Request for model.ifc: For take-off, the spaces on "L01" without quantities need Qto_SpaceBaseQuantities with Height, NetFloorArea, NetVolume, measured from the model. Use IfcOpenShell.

First a look at what the model holds.

```python
import ifcopenshell
import ifcopenshell.util.element
import ifcopenshell.util.unit

model = ifcopenshell.open("model.ifc")
print(model.schema)
for unit_type in ("LENGTHUNIT", "AREAUNIT", "VOLUMEUNIT"):
    print(unit_type, ifcopenshell.util.unit.calculate_unit_scale(model, unit_type))
storey = next(s for s in model.by_type("IfcBuildingStorey") if s.Name == "L01")
spaces = [e for e in ifcopenshell.util.element.get_decomposition(storey) if e.is_a("IfcSpace")]
for e in sorted(spaces, key=lambda e: e.id()):
    print(e.id(), e.is_a(), e.Name, list(ifcopenshell.util.element.get_psets(e, qtos_only=True)), sep=" | ")
```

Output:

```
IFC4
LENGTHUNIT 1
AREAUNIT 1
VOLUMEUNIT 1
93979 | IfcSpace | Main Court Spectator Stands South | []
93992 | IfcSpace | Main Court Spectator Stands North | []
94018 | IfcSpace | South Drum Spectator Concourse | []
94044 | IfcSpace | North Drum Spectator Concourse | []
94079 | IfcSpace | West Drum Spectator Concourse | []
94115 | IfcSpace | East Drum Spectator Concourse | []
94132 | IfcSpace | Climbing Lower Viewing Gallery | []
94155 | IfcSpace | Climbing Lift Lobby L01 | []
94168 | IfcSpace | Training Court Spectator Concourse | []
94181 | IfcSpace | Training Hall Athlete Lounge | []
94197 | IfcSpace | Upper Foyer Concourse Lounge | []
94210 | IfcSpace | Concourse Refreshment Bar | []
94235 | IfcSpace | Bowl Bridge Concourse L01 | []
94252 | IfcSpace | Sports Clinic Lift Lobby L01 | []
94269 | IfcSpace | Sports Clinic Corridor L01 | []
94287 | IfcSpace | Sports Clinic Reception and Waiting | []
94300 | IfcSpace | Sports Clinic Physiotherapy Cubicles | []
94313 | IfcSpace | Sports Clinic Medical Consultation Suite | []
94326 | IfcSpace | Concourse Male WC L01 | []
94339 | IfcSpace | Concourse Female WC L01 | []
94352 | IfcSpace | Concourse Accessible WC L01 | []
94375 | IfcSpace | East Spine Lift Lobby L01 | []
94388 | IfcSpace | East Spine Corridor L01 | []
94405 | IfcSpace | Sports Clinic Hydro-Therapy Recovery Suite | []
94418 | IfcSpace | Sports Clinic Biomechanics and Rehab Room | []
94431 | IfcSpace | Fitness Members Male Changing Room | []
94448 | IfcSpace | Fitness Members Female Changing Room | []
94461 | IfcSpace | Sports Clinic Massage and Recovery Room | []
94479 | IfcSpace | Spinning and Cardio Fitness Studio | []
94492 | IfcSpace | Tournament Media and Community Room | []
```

```python
import ifcopenshell
import ifcopenshell.api.pset
import ifcopenshell.geom
import ifcopenshell.util.element
import ifcopenshell.util.shape
import ifcopenshell.util.unit

model = ifcopenshell.open("model.ifc")
unit_scale = ifcopenshell.util.unit.calculate_unit_scale(model)
area_scale = ifcopenshell.util.unit.calculate_unit_scale(model, "AREAUNIT")
volume_scale = ifcopenshell.util.unit.calculate_unit_scale(model, "VOLUMEUNIT")
settings = ifcopenshell.geom.settings()

storey = next(s for s in model.by_type("IfcBuildingStorey") if s.Name == "L01")
spaces = [e for e in ifcopenshell.util.element.get_decomposition(storey) if e.is_a("IfcSpace")]

for e in sorted(spaces, key=lambda e: e.id()):
    if ifcopenshell.util.element.get_psets(e, qtos_only=True, should_inherit=False):
        continue
    # Geometry comes back in metres, in the element's own axes.
    shape = ifcopenshell.geom.create_shape(settings, e)
    values = {
        "Height": ifcopenshell.util.shape.get_z(shape.geometry) / unit_scale,
        "NetFloorArea": ifcopenshell.util.shape.get_footprint_area(shape.geometry) / area_scale,
        "NetVolume": ifcopenshell.util.shape.get_volume(shape.geometry) / volume_scale,
    }
    qto = ifcopenshell.api.pset.add_qto(model, product=e, name="Qto_SpaceBaseQuantities")
    ifcopenshell.api.pset.edit_qto(model, qto=qto, properties=values)
    print(e.id(), {k: round(v, 3) for k, v in values.items()})

model.write("model_edited.ifc")
```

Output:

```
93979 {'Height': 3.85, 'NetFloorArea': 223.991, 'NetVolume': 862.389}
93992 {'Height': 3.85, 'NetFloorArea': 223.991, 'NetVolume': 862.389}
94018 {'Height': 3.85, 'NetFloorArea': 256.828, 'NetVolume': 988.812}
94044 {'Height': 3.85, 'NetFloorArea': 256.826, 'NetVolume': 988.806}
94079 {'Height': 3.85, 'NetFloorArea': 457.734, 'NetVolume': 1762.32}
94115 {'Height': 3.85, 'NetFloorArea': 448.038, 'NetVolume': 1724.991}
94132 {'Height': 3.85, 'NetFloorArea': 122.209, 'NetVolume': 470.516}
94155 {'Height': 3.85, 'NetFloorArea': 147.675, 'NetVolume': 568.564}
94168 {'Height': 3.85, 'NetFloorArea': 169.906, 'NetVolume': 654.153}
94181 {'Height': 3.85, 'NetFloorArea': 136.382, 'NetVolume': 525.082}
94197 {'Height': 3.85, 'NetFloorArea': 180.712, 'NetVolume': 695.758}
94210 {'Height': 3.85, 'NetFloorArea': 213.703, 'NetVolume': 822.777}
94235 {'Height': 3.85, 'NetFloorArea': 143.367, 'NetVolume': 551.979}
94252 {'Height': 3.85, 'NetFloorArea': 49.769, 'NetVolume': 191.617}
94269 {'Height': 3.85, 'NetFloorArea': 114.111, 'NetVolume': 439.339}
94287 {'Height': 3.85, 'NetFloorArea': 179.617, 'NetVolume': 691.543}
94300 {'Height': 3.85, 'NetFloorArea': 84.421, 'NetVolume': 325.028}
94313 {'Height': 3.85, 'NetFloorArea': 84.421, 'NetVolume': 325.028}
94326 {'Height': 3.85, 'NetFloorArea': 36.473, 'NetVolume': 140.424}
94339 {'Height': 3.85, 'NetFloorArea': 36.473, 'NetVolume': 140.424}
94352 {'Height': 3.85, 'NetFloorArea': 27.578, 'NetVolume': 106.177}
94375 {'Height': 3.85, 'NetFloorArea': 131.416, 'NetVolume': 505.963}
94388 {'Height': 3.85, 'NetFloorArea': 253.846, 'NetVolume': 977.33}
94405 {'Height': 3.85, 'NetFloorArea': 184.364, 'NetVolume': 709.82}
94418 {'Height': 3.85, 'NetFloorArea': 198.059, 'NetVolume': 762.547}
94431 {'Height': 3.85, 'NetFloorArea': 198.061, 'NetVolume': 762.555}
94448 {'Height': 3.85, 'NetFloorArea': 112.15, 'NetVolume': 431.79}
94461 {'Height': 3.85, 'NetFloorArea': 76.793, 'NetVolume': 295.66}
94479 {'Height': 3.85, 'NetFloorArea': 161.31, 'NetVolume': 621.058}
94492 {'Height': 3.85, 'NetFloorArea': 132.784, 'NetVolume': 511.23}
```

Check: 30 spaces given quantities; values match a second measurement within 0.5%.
